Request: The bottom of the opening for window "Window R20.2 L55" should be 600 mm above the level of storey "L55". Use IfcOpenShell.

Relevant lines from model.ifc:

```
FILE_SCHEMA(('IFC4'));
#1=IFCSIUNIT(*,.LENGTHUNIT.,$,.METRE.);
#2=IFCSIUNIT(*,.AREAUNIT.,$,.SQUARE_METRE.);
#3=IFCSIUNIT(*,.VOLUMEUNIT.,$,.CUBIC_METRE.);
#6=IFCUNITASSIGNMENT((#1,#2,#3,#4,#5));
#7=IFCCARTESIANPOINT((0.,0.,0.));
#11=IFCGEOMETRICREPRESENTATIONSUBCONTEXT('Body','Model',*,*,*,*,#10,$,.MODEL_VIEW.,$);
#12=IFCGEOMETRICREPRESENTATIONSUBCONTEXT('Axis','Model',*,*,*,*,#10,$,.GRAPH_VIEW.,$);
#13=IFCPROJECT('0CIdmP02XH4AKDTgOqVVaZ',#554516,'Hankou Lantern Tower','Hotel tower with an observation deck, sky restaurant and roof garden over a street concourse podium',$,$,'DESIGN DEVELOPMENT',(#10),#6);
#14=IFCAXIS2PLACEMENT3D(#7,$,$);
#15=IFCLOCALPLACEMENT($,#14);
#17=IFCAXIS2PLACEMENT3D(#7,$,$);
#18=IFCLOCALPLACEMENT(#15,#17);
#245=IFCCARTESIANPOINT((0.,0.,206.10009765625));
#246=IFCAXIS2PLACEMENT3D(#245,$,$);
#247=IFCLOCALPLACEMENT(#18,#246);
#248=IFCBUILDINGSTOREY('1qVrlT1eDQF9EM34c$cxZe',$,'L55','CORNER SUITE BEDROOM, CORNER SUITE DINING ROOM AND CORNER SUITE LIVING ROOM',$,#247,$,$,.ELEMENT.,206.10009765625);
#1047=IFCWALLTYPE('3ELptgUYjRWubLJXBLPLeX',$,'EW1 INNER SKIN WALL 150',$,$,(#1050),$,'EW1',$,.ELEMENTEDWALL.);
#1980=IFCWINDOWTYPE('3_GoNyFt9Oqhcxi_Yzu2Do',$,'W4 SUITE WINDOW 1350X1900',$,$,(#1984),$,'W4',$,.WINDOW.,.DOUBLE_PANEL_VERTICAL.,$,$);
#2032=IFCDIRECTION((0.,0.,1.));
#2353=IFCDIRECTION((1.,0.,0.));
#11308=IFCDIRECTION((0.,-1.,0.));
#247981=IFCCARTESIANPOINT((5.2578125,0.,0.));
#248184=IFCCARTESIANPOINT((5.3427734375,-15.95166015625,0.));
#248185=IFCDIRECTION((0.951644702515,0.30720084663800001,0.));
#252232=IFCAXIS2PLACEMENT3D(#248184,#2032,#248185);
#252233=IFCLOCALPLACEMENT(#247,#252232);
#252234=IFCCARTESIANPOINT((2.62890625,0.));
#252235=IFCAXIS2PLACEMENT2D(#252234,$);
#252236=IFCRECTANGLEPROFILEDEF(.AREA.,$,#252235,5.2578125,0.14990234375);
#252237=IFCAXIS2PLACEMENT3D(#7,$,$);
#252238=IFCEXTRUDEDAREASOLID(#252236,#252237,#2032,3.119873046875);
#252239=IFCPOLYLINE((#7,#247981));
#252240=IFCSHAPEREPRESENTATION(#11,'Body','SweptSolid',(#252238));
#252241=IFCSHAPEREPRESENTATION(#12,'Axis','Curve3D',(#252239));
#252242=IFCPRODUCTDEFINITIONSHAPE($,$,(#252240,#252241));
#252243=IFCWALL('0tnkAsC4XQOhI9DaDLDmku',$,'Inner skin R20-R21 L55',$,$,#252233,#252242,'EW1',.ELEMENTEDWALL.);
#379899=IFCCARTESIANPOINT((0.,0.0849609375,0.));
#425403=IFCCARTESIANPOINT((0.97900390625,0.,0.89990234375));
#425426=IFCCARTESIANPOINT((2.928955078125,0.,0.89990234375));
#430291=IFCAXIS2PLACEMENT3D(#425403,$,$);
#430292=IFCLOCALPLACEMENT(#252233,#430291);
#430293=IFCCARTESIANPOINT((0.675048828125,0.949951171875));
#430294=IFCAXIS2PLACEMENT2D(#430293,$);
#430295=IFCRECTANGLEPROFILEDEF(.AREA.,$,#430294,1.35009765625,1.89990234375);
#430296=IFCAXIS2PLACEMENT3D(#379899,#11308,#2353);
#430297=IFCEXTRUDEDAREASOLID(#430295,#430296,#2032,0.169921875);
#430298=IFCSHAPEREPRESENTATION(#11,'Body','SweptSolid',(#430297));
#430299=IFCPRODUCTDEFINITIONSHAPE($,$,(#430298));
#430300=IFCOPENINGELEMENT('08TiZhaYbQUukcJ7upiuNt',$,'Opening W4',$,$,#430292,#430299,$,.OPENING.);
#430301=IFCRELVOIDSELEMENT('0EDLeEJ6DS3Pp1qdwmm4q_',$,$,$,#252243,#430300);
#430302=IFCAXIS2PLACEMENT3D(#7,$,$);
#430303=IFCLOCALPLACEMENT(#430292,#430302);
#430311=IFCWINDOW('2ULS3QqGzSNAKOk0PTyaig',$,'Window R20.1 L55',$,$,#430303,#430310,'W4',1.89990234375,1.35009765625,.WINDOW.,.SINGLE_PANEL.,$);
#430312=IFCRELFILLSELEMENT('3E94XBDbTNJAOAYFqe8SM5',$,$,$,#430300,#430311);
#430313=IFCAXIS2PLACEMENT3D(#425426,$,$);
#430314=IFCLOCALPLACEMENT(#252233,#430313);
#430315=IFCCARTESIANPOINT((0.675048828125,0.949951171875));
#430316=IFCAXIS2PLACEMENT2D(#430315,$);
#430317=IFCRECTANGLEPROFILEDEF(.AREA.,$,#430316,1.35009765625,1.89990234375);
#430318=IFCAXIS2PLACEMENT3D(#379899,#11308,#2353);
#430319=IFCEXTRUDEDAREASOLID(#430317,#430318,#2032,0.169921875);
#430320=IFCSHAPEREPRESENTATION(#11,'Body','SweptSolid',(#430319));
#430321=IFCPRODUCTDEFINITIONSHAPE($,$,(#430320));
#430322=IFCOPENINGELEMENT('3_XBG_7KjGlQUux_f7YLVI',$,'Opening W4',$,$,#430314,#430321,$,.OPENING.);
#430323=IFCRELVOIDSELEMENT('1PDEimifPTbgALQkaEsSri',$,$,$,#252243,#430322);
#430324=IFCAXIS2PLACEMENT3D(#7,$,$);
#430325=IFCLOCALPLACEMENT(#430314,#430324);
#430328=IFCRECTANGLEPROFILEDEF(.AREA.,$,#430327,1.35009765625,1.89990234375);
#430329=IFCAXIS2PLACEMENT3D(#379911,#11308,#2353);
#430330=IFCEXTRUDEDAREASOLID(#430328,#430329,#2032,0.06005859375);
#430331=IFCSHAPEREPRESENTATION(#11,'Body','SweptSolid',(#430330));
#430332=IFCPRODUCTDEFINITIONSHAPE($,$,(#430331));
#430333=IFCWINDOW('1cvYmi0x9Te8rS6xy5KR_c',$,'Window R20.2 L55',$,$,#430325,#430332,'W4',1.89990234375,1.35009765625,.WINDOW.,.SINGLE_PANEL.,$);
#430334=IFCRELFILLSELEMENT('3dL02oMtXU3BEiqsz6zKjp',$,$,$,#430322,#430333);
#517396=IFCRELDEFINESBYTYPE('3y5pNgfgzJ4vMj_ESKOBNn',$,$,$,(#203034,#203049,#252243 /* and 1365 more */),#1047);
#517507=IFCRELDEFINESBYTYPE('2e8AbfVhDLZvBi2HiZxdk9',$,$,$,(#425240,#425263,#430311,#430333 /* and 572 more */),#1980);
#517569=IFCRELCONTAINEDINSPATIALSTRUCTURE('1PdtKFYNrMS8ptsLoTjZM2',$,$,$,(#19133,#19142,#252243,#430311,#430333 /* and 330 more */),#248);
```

```python
import numpy as np
import ifcopenshell
import ifcopenshell.api.geometry
import ifcopenshell.geom
import ifcopenshell.util.element
import ifcopenshell.util.placement
import ifcopenshell.util.shape
import ifcopenshell.util.unit

model = ifcopenshell.open("model.ifc")
unit_scale = ifcopenshell.util.unit.calculate_unit_scale(model)

window = model.by_id(430333)
opening = window.FillsVoids[0].RelatingOpeningElement
storey = ifcopenshell.util.element.get_container(window, ifc_class="IfcBuildingStorey")
level = ifcopenshell.util.placement.get_local_placement(storey.ObjectPlacement)[2, 3]

# The opening's origin need not be at the sill, so measure its lowest point.
shape = ifcopenshell.geom.create_shape(ifcopenshell.geom.settings(), opening)
bottom = ifcopenshell.util.shape.get_shape_bottom_elevation(shape, shape.geometry) / unit_scale
dz = level + 0.6 - bottom

shift = np.array([0.0, 0.0, dz])
# The window is placed relative to its opening, so it follows when the opening moves.
matrix = ifcopenshell.util.placement.get_local_placement(opening.ObjectPlacement)
matrix[:3, 3] += shift
ifcopenshell.api.geometry.edit_object_placement(
    model, product=opening, matrix=matrix, is_si=False, should_transform_children=True
)

print(f"moved by {dz * unit_scale:+.3f} m")

model.write("model_rev.ifc")
```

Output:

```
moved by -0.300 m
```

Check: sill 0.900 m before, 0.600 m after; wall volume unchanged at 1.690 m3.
